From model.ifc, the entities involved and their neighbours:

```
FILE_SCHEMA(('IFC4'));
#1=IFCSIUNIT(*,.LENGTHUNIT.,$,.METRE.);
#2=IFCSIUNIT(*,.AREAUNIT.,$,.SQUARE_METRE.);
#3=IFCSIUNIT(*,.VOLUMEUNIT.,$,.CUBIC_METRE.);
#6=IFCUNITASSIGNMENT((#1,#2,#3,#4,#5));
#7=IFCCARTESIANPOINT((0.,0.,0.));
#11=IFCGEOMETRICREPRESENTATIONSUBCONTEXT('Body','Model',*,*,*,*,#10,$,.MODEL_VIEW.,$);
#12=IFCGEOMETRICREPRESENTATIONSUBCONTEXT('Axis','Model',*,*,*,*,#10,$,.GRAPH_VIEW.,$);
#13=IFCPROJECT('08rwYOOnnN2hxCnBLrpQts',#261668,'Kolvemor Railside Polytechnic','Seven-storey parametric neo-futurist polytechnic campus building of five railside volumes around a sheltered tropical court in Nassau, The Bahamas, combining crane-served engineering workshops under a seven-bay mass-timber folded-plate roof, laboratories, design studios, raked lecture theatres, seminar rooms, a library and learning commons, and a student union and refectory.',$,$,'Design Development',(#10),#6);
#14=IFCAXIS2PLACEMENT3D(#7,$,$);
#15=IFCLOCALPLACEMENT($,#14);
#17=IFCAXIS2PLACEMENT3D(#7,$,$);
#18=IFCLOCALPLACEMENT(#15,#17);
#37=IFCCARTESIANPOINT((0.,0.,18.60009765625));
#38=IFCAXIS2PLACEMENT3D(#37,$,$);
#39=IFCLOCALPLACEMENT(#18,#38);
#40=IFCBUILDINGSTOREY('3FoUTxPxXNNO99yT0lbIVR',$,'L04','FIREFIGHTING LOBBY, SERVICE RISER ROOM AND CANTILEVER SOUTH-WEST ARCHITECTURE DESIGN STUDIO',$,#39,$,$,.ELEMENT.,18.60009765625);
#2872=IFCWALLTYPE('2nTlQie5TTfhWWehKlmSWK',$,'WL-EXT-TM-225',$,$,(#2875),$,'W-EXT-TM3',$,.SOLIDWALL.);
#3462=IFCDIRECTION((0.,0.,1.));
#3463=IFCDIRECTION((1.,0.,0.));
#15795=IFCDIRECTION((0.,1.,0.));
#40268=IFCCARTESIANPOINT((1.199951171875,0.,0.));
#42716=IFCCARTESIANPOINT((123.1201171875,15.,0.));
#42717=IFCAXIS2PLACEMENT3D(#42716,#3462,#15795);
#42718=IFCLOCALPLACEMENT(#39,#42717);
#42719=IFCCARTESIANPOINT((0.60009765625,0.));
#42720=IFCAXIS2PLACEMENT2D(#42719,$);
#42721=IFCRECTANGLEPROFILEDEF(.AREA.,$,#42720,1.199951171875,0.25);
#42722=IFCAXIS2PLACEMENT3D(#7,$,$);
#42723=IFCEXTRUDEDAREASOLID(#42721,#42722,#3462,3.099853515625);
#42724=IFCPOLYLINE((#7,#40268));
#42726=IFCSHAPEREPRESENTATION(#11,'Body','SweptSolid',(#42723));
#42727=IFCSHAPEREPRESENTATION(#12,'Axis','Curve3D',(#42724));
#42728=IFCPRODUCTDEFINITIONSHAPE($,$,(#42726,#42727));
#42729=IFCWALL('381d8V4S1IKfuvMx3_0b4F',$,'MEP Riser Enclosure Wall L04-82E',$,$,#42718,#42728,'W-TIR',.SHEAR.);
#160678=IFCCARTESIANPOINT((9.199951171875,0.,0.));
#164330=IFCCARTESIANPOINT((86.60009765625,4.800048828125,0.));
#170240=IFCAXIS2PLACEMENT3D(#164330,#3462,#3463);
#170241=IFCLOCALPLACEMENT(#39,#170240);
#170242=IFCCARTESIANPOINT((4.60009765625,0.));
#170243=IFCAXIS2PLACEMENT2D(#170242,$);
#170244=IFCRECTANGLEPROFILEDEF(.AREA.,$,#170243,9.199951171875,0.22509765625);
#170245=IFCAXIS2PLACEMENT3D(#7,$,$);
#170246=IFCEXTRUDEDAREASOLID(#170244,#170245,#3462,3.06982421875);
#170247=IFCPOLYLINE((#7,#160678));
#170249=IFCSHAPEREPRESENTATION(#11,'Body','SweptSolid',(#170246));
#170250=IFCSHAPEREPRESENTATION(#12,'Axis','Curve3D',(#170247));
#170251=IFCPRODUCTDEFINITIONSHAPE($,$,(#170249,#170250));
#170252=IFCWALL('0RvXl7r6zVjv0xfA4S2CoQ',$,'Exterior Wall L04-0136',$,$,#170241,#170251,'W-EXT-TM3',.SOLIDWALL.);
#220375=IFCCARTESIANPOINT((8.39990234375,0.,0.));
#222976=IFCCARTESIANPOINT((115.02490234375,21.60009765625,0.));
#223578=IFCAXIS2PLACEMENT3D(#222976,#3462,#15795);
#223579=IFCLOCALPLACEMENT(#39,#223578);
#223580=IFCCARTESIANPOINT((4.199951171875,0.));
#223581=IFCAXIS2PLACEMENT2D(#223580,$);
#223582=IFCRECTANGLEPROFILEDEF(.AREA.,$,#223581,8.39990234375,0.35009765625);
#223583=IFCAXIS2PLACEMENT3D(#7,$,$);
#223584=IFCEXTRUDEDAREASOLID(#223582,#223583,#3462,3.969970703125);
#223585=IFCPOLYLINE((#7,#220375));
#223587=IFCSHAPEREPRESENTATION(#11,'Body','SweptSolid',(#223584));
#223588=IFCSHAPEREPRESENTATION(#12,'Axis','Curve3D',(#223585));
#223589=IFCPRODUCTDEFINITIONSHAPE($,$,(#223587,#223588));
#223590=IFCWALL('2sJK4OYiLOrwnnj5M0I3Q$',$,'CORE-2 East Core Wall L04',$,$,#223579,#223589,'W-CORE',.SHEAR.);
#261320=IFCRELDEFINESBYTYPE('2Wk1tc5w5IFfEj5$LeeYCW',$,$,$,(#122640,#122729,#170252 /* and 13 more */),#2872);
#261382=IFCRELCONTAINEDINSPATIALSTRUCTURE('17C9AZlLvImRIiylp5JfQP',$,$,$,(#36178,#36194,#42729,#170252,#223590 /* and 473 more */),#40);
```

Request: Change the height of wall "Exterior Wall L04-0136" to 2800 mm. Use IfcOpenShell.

```python
import ifcopenshell
import ifcopenshell.geom
import ifcopenshell.util.representation
import ifcopenshell.util.shape
import ifcopenshell.util.unit

model = ifcopenshell.open("model.ifc")
unit_scale = ifcopenshell.util.unit.calculate_unit_scale(model)
settings = ifcopenshell.geom.settings()


def volume(element):
    """Net volume in cubic metres, openings subtracted."""
    shape = ifcopenshell.geom.create_shape(settings, element)
    return ifcopenshell.util.shape.get_volume(shape.geometry)


wall = model.by_guid("0RvXl7r6zVjv0xfA4S2CoQ")
before = volume(wall)

body = ifcopenshell.util.representation.get_representation(wall, "Model", "Body")
solid = body.Items[0]
old_height = solid.Depth
solid.Depth = 2.8 / unit_scale
after = volume(wall)

print(f"height {old_height:g} -> {solid.Depth:g}, volume {before:.3f} -> {after:.3f} m3")

model.write("model_updated.ifc")
```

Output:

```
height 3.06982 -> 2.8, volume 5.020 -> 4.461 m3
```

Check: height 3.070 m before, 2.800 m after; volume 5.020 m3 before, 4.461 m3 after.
